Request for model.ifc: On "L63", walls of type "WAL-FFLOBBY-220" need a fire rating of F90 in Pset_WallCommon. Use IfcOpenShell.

First a look at what the model holds.

```python
import ifcopenshell
import ifcopenshell.util.element

model = ifcopenshell.open("model.ifc")
print(model.schema)
storey = next(s for s in model.by_type("IfcBuildingStorey") if s.Name == "L63")
walls = [e for e in ifcopenshell.util.element.get_decomposition(storey) if e.is_a("IfcWall")]
seen = {}
for e in walls:
    element_type = ifcopenshell.util.element.get_type(e)
    key = (element_type.Name if element_type != e and element_type else None, ifcopenshell.util.element.get_pset(e, "Pset_WallCommon", "FireRating"))
    seen[key] = seen.get(key, 0) + 1
for (name, value), count in sorted(seen.items(), key=str):
    print(count, "x", name, "|", value)
```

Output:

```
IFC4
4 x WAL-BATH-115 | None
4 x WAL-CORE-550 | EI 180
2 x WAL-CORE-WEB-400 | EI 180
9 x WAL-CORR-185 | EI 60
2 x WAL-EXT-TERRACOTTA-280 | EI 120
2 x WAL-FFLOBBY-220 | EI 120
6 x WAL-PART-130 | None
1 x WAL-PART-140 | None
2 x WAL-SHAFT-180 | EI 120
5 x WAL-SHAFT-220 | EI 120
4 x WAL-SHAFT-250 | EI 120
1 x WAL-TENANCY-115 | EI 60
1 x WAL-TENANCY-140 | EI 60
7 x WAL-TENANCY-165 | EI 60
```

```python
import ifcopenshell
import ifcopenshell.api.pset
import ifcopenshell.util.element

model = ifcopenshell.open("model.ifc")

storey = next(s for s in model.by_type("IfcBuildingStorey") if s.Name == "L63")
walls = [e for e in ifcopenshell.util.element.get_decomposition(storey) if e.is_a("IfcWall")]

count = 0
for e in walls:
    element_type = ifcopenshell.util.element.get_type(e)
    if element_type in (None, e) or element_type.Name != "WAL-FFLOBBY-220":
        continue
    found = ifcopenshell.util.element.get_pset(e, "Pset_WallCommon", should_inherit=False)
    if found:
        pset = model.by_id(found["id"])
        if len(ifcopenshell.util.element.get_elements_by_pset(pset)) > 1:
            pset = ifcopenshell.api.pset.unshare_pset(model, products=[e], pset=pset)[0]
    else:
        pset = ifcopenshell.api.pset.add_pset(model, product=e, name="Pset_WallCommon")
    ifcopenshell.api.pset.edit_pset(model, pset=pset, properties={"FireRating": "F90"})
    count += 1

print(count, "walls updated")

model.write("model-out.ifc")
```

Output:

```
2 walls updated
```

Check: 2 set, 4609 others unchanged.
